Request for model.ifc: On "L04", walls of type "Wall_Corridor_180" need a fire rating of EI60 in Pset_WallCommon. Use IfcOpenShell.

First a look at what the model holds.

```python
import ifcopenshell
import ifcopenshell.util.element

model = ifcopenshell.open("model.ifc")
print(model.schema)
storey = next(s for s in model.by_type("IfcBuildingStorey") if s.Name == "L04")
walls = [e for e in ifcopenshell.util.element.get_decomposition(storey) if e.is_a("IfcWall")]
seen = {}
for e in walls:
    element_type = ifcopenshell.util.element.get_type(e)
    key = (element_type.Name if element_type != e and element_type else None, ifcopenshell.util.element.get_pset(e, "Pset_WallCommon", "FireRating"))
    seen[key] = seen.get(key, 0) + 1
for (name, value), count in sorted(seen.items(), key=str):
    print(count, "x", name, "|", value)
```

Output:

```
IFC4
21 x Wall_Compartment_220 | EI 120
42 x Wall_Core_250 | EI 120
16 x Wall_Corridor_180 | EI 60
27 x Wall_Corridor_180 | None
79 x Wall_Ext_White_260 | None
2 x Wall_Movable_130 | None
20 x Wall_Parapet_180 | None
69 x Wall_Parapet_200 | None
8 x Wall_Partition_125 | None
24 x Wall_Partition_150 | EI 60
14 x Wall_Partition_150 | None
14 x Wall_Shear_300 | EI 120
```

```python
import ifcopenshell
import ifcopenshell.api.pset
import ifcopenshell.util.element

model = ifcopenshell.open("model.ifc")

storey = next(s for s in model.by_type("IfcBuildingStorey") if s.Name == "L04")
walls = [e for e in ifcopenshell.util.element.get_decomposition(storey) if e.is_a("IfcWall")]

count = 0
for e in walls:
    element_type = ifcopenshell.util.element.get_type(e)
    if element_type in (None, e) or element_type.Name != "Wall_Corridor_180":
        continue
    # add_pset returns the element's existing set when there is one.
    pset = ifcopenshell.api.pset.add_pset(model, product=e, name="Pset_WallCommon")
    ifcopenshell.api.pset.edit_pset(model, pset=pset, properties={"FireRating": "EI60"})
    count += 1

print(count, "walls updated")

model.write("model_v2.ifc")
```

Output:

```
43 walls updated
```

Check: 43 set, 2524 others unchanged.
